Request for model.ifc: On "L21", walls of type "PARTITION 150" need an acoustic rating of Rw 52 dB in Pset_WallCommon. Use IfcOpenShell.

First a look at what the model holds.

```python
import ifcopenshell
import ifcopenshell.util.element

model = ifcopenshell.open("model.ifc")
print(model.schema)
storey = next(s for s in model.by_type("IfcBuildingStorey") if s.Name == "L21")
walls = [e for e in ifcopenshell.util.element.get_decomposition(storey) if e.is_a("IfcWall")]
seen = {}
for e in walls:
    element_type = ifcopenshell.util.element.get_type(e)
    key = (element_type.Name if element_type != e and element_type else None, ifcopenshell.util.element.get_pset(e, "Pset_WallCommon", "AcousticRating"))
    seen[key] = seen.get(key, 0) + 1
for (name, value), count in sorted(seen.items(), key=str):
    print(count, "x", name, "|", value)
```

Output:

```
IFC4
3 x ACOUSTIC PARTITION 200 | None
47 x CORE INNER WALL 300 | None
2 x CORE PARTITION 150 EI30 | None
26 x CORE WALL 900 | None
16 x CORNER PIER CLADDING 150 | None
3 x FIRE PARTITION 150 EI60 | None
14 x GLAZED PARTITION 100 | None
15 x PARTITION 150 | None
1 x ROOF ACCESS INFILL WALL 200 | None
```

```python
import ifcopenshell
import ifcopenshell.api.pset
import ifcopenshell.util.element

model = ifcopenshell.open("model.ifc")

storey = next(s for s in model.by_type("IfcBuildingStorey") if s.Name == "L21")
walls = [e for e in ifcopenshell.util.element.get_decomposition(storey) if e.is_a("IfcWall")]

count = 0
for e in walls:
    element_type = ifcopenshell.util.element.get_type(e)
    if element_type in (None, e) or element_type.Name != "PARTITION 150":
        continue
    found = ifcopenshell.util.element.get_pset(e, "Pset_WallCommon", should_inherit=False)
    if found:
        pset = model.by_id(found["id"])
        if len(ifcopenshell.util.element.get_elements_by_pset(pset)) > 1:
            pset = ifcopenshell.api.pset.unshare_pset(model, products=[e], pset=pset)[0]
    else:
        pset = ifcopenshell.api.pset.add_pset(model, product=e, name="Pset_WallCommon")
    ifcopenshell.api.pset.edit_pset(model, pset=pset, properties={"AcousticRating": "Rw 52 dB"})
    count += 1

print(count, "walls updated")

model.write("model_edited.ifc")
```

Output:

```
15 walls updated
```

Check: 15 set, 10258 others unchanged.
